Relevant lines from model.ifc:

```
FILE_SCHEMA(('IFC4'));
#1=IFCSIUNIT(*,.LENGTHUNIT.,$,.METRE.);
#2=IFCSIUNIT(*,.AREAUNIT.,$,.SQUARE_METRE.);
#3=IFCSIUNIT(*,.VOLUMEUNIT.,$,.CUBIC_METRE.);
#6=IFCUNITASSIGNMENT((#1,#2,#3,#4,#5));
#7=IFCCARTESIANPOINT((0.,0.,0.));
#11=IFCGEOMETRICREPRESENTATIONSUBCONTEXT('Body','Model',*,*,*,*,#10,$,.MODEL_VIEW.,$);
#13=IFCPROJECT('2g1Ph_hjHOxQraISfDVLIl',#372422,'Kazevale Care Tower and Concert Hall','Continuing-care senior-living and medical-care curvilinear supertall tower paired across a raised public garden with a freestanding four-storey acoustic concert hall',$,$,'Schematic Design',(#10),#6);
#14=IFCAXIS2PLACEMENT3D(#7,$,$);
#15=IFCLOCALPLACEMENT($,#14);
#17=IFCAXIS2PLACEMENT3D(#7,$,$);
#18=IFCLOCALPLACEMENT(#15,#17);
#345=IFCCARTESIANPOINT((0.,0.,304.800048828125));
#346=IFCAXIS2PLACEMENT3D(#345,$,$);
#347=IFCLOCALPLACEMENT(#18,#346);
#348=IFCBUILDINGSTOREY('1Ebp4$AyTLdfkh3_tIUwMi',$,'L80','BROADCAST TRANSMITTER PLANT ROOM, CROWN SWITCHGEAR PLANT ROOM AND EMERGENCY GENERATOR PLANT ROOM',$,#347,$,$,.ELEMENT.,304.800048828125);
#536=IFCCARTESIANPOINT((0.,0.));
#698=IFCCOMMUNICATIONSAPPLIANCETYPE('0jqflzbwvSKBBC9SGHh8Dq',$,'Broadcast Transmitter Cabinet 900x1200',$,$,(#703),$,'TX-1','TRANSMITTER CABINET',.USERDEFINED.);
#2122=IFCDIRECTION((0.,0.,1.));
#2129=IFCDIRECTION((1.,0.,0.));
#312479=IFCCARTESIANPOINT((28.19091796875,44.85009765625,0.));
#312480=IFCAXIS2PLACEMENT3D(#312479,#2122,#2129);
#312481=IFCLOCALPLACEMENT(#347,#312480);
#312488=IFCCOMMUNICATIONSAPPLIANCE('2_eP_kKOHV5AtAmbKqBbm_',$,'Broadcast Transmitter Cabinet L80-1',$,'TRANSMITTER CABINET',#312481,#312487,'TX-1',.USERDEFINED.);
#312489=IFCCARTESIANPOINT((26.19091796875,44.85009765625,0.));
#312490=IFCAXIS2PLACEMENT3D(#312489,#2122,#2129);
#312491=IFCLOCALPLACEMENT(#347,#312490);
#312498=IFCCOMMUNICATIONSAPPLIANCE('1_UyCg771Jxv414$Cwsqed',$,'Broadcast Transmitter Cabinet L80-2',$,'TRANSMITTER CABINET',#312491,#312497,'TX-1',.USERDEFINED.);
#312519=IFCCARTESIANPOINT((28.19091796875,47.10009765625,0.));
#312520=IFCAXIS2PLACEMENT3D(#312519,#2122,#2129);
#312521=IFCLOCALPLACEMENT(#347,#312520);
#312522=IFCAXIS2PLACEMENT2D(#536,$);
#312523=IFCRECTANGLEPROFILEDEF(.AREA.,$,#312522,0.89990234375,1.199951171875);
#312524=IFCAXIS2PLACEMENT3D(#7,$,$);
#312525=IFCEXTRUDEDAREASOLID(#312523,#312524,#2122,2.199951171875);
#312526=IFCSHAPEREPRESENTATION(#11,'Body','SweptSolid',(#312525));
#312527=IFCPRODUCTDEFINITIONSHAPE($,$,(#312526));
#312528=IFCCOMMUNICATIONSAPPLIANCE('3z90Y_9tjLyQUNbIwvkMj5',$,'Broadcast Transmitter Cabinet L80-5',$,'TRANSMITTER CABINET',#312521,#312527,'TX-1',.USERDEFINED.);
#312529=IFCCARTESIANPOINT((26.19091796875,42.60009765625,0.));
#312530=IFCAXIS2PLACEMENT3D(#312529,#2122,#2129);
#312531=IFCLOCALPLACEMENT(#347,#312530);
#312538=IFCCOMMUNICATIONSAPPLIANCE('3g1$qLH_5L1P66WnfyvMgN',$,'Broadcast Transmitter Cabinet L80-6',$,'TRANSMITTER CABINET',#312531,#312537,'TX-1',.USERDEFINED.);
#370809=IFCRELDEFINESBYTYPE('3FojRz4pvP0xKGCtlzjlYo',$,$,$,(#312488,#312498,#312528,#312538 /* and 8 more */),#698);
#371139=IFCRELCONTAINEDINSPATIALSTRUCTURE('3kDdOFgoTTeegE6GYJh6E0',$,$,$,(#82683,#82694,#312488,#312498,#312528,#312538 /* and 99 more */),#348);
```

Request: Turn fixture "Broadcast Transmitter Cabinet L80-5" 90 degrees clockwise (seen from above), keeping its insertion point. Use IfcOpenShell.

```python
import ifcopenshell
import ifcopenshell.api.geometry
import ifcopenshell.util.placement

model = ifcopenshell.open("model.ifc")

item = model.by_id(312528)
matrix = ifcopenshell.util.placement.get_local_placement(item.ObjectPlacement)
matrix = matrix @ ifcopenshell.util.placement.rotation(-90, "Z")
ifcopenshell.api.geometry.edit_object_placement(model, product=item, matrix=matrix, is_si=False)

print(ifcopenshell.util.placement.get_local_placement(item.ObjectPlacement).round(3) + 0.0)

model.write("model_updated.ifc")
```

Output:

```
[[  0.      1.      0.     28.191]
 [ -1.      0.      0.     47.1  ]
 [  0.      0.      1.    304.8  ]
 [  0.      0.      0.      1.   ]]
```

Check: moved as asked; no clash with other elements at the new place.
